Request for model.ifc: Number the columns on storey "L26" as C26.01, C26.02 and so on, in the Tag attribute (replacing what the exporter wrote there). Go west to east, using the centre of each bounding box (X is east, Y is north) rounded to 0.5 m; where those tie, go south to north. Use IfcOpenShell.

First a look at what the model holds.

```python
import ifcopenshell
import ifcopenshell.util.element
import ifcopenshell.util.placement

model = ifcopenshell.open("model.ifc")
print(model.schema)
storey = next(s for s in model.by_type("IfcBuildingStorey") if s.Name == "L26")
columns = [e for e in ifcopenshell.util.element.get_decomposition(storey) if e.is_a("IfcColumn")]
for e in sorted(columns, key=lambda e: e.id()):
    origin = ifcopenshell.util.placement.get_local_placement(e.ObjectPlacement)[:3, 3]
    print(e.id(), e.Tag, e.Name, origin.round(2) + 0.0, sep=" | ")
```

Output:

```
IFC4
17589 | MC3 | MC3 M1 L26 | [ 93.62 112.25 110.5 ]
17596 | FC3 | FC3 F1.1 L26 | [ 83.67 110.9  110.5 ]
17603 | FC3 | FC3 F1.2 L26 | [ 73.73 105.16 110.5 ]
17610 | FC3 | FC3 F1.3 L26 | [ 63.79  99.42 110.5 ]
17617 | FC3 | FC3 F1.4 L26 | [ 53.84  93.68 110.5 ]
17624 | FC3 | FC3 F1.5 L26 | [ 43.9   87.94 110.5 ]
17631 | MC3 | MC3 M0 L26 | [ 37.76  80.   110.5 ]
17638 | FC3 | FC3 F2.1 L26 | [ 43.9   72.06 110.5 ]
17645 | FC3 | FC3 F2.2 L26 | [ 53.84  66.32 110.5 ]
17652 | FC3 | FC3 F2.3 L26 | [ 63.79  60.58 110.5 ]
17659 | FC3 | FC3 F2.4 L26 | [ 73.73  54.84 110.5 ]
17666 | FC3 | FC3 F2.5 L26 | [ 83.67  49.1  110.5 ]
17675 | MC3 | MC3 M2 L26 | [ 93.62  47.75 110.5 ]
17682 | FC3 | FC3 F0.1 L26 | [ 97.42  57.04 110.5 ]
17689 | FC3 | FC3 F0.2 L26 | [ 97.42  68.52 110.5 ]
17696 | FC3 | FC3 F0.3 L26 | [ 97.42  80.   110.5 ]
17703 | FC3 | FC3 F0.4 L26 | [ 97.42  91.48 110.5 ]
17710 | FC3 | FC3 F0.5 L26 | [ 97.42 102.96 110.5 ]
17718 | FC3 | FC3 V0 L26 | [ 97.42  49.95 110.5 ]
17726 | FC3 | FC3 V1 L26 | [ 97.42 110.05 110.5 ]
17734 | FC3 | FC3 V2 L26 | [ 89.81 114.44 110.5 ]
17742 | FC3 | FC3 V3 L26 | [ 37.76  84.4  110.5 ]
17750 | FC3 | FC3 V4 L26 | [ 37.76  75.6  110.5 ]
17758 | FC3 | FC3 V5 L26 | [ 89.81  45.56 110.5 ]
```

```python
import ifcopenshell
import ifcopenshell.geom
import ifcopenshell.util.element
import ifcopenshell.util.shape

model = ifcopenshell.open("model.ifc")
settings = ifcopenshell.geom.settings()
settings.set("use-world-coords", True)


def centre(element):
    shape = ifcopenshell.geom.create_shape(settings, element)
    return ifcopenshell.util.shape.get_bbox_centroid(shape.geometry)


storey = next(s for s in model.by_type("IfcBuildingStorey") if s.Name == "L26")
columns = [e for e in ifcopenshell.util.element.get_decomposition(storey) if e.is_a("IfcColumn")]

# Insertion points can sit at a corner or the storey origin, so sort by the geometry (in metres).
centres = {e: centre(e) for e in columns}
columns.sort(key=lambda e: (round(centres[e][0] / 0.5), centres[e][1]))

for i, e in enumerate(columns, start=1):
    number = f"C26.{i:02d}"
    e.Tag = number
    print(e.id(), number)

model.write("model_v2.ifc")
```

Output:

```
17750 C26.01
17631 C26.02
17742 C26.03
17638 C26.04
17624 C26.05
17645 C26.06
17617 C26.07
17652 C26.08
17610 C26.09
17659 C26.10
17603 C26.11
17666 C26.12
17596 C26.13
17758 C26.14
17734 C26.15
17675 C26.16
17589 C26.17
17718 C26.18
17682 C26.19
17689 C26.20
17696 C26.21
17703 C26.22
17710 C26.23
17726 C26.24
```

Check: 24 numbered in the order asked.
